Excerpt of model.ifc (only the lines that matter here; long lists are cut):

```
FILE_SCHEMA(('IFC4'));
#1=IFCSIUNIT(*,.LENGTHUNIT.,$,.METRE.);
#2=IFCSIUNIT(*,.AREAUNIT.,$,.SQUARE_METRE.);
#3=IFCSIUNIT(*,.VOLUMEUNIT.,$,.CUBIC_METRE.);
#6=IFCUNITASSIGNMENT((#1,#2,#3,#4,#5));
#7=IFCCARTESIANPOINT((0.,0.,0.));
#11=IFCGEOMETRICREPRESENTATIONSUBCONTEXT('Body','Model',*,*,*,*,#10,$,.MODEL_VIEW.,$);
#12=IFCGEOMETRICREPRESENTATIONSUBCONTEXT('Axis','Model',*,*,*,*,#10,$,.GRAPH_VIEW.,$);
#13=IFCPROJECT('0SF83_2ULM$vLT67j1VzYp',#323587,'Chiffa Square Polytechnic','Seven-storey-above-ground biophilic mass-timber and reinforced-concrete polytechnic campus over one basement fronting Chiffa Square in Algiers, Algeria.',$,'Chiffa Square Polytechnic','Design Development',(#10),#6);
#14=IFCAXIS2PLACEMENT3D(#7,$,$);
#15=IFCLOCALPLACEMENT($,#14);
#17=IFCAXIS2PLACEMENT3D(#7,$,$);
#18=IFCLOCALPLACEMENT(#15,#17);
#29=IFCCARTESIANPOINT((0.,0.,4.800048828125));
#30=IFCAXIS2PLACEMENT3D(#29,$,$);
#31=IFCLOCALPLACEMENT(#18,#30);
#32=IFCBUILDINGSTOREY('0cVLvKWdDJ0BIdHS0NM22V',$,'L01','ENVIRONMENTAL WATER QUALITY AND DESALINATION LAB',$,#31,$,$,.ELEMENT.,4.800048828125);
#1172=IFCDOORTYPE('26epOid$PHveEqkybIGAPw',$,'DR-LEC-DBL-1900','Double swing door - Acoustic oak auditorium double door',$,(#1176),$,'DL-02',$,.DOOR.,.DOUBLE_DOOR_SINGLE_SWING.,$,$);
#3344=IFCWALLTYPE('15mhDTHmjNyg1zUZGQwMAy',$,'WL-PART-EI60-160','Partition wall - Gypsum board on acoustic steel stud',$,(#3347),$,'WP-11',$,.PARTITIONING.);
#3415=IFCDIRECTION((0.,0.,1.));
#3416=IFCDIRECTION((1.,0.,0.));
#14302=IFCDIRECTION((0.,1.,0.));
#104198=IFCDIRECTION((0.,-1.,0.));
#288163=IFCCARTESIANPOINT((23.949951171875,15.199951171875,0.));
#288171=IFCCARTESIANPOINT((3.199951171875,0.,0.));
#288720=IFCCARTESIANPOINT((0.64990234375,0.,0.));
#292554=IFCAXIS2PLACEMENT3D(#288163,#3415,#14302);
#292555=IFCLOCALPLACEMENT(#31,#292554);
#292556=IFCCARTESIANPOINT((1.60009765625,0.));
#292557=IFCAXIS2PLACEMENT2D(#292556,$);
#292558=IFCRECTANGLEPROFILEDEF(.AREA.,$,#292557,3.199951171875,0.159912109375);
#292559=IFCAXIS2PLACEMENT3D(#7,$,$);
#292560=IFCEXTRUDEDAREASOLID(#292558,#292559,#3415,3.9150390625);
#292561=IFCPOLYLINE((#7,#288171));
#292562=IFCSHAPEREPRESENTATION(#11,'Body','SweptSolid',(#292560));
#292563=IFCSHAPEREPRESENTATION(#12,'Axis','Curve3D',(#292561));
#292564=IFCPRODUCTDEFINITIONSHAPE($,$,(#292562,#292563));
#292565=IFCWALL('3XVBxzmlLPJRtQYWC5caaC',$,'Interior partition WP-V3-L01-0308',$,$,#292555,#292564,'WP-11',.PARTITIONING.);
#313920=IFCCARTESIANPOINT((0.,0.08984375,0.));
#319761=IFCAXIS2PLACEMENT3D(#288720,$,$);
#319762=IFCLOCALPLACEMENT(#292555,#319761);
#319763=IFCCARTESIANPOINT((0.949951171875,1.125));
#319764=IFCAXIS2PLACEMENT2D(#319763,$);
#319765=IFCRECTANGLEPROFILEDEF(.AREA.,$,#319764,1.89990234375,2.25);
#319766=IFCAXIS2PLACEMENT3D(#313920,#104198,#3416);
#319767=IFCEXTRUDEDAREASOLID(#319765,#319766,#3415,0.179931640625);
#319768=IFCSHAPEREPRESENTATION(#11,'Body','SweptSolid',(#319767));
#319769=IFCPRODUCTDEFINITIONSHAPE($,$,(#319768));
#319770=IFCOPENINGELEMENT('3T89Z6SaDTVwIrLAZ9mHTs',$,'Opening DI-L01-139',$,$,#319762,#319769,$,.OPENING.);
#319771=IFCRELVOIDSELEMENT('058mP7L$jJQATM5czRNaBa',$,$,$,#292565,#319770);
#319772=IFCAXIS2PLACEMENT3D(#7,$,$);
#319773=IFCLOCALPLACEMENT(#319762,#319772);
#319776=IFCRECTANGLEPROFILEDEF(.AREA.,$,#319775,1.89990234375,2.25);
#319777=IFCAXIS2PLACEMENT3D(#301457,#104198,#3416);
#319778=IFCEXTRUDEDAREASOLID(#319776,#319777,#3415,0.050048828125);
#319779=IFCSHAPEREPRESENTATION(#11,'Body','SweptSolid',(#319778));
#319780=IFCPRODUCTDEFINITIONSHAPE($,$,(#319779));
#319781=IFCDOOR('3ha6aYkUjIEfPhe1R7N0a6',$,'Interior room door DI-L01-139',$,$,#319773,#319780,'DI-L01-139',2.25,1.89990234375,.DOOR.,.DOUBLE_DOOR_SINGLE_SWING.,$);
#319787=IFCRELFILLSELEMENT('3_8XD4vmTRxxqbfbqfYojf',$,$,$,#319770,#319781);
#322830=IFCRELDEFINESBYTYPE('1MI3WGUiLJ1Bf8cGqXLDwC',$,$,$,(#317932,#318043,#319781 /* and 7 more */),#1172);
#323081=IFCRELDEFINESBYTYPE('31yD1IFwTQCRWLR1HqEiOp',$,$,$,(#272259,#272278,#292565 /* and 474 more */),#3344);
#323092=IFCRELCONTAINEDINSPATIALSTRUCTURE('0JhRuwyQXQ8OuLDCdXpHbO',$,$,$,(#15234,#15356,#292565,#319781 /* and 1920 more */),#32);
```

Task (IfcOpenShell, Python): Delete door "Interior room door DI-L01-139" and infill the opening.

```python
import ifcopenshell
import ifcopenshell.api.feature
import ifcopenshell.api.root
import ifcopenshell.geom
import ifcopenshell.util.shape

model = ifcopenshell.open("model.ifc")
settings = ifcopenshell.geom.settings()


def volume(element):
    """Net volume in cubic metres, openings subtracted."""
    shape = ifcopenshell.geom.create_shape(settings, element)
    return ifcopenshell.util.shape.get_volume(shape.geometry)


door = model.by_id(319781)
opening = door.FillsVoids[0].RelatingOpeningElement
wall = opening.VoidsElements[0].RelatingBuildingElement
before = volume(wall)

ifcopenshell.api.root.remove_product(model, product=door)
ifcopenshell.api.feature.remove_feature(model, feature=opening)

after = volume(wall)

print(f"wall volume {before:.3f} -> {after:.3f} m3")

model.write("model-out.ifc")
```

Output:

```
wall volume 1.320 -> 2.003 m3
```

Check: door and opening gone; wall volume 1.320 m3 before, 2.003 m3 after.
